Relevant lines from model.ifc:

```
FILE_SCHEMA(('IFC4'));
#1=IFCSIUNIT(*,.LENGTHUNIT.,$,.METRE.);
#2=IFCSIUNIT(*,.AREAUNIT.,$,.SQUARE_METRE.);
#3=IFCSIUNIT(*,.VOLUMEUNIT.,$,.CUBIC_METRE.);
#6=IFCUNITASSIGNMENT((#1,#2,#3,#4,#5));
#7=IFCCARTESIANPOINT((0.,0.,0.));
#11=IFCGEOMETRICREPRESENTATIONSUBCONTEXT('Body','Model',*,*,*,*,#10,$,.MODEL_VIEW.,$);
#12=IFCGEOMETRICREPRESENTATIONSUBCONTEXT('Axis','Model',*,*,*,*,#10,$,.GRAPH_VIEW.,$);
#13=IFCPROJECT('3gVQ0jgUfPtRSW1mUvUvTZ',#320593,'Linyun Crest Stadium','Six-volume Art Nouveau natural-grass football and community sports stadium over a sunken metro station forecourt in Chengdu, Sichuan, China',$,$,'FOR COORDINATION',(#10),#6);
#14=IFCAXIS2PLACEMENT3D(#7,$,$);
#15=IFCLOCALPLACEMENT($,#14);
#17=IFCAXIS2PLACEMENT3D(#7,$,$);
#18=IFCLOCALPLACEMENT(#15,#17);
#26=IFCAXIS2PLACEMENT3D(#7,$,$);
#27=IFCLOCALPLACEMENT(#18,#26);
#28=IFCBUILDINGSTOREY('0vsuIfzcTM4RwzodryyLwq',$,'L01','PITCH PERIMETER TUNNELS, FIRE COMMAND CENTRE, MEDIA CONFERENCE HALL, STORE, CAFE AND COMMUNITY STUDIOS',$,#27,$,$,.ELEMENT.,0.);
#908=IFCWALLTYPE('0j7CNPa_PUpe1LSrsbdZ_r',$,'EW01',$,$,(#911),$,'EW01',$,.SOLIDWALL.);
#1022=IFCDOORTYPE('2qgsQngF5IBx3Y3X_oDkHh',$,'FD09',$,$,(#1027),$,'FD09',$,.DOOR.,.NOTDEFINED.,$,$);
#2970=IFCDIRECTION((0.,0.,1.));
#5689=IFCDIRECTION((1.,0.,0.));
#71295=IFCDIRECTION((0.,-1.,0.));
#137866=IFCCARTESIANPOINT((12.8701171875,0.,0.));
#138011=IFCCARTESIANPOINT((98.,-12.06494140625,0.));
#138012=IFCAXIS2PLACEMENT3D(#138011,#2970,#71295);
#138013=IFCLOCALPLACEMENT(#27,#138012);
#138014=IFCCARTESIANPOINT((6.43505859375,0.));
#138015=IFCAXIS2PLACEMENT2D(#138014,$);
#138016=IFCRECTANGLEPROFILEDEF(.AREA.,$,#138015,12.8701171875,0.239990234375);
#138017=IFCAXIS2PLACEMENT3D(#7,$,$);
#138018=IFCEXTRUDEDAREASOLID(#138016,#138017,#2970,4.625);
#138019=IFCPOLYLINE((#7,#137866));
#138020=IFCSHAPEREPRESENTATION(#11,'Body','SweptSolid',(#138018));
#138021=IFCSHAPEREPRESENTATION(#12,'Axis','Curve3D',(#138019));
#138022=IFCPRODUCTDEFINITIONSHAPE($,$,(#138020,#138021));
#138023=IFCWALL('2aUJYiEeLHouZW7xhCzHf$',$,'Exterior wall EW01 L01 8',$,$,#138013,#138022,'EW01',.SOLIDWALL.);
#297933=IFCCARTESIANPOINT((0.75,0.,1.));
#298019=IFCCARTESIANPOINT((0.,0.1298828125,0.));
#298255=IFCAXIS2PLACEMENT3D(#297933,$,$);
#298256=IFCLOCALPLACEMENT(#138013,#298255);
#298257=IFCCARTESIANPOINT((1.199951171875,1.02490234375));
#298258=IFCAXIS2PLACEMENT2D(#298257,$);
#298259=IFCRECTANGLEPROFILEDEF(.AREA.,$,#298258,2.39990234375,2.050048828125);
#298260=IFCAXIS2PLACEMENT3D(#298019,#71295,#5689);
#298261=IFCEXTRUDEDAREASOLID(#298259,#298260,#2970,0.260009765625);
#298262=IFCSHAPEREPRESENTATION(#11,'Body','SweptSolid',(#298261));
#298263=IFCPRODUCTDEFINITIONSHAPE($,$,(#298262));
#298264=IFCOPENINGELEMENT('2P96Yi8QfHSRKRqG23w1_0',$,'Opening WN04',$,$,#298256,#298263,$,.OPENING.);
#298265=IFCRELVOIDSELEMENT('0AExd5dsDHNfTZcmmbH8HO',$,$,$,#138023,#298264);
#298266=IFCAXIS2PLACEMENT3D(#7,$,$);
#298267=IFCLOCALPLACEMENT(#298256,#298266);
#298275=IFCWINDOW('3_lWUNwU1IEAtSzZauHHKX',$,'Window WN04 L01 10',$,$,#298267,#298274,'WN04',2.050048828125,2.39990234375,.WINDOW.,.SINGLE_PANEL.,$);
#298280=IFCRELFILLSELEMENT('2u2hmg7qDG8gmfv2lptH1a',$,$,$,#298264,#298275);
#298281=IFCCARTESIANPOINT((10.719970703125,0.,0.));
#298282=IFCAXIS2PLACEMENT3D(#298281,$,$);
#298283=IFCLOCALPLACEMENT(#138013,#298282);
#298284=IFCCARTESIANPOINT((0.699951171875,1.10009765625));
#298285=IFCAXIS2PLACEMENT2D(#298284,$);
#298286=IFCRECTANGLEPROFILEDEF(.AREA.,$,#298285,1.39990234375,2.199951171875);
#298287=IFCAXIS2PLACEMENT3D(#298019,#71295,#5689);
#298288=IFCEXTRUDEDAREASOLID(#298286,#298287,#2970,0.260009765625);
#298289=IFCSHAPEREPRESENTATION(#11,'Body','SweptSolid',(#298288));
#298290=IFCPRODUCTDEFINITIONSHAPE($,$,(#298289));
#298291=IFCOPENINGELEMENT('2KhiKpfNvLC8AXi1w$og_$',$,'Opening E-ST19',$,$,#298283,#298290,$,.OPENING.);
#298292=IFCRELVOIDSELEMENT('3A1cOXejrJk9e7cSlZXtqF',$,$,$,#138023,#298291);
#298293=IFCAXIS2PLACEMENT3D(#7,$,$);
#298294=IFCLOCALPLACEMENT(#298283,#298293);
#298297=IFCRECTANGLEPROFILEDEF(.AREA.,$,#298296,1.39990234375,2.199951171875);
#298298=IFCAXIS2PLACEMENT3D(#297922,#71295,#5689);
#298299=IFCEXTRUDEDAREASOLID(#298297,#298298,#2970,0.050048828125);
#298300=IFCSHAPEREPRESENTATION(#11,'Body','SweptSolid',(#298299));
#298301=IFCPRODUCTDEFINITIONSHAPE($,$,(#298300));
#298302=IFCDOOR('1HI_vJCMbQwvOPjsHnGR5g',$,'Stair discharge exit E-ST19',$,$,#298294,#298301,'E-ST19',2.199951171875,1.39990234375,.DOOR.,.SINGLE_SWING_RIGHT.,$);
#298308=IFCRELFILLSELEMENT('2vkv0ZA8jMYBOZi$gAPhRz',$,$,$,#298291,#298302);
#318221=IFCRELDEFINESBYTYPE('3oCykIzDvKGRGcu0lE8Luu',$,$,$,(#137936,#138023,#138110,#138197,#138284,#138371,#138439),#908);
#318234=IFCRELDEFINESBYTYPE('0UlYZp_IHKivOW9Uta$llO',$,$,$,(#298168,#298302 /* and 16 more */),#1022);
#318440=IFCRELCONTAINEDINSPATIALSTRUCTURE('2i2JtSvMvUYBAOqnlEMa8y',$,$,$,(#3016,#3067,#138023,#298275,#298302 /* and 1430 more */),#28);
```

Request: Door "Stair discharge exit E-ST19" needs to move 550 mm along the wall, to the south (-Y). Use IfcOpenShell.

```python
import ifcopenshell
import ifcopenshell.api.geometry
import ifcopenshell.util.placement
import ifcopenshell.util.unit

model = ifcopenshell.open("model.ifc")
unit_scale = ifcopenshell.util.unit.calculate_unit_scale(model)

door = model.by_guid("1HI_vJCMbQwvOPjsHnGR5g")
opening = door.FillsVoids[0].RelatingOpeningElement
wall = opening.VoidsElements[0].RelatingBuildingElement

wall_matrix = ifcopenshell.util.placement.get_local_placement(wall.ObjectPlacement)
shift = wall_matrix[:3, 0] * 0.55 / unit_scale
before = ifcopenshell.util.placement.get_local_placement(door.ObjectPlacement)[:3, 3].copy()

# The door is placed relative to its opening, so it follows when the opening moves.
matrix = ifcopenshell.util.placement.get_local_placement(opening.ObjectPlacement)
matrix[:3, 3] += shift
ifcopenshell.api.geometry.edit_object_placement(
    model, product=opening, matrix=matrix, is_si=False, should_transform_children=True
)

after = ifcopenshell.util.placement.get_local_placement(door.ObjectPlacement)[:3, 3]
print("door moved by", (after - before).round(3) + 0.0)

model.write("model_v2.ifc")
```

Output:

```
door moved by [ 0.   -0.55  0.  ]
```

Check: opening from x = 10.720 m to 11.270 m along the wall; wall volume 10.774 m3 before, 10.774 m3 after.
